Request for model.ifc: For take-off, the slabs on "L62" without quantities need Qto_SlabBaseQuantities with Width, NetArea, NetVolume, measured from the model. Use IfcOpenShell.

First a look at what the model holds.

```python
import ifcopenshell
import ifcopenshell.util.element
import ifcopenshell.util.unit

model = ifcopenshell.open("model.ifc")
print(model.schema)
for unit_type in ("LENGTHUNIT", "AREAUNIT", "VOLUMEUNIT"):
    print(unit_type, ifcopenshell.util.unit.calculate_unit_scale(model, unit_type))
storey = next(s for s in model.by_type("IfcBuildingStorey") if s.Name == "L62")
slabs = [e for e in ifcopenshell.util.element.get_decomposition(storey) if e.is_a("IfcSlab")]
for e in sorted(slabs, key=lambda e: e.id()):
    print(e.id(), e.is_a(), e.Name, list(ifcopenshell.util.element.get_psets(e, qtos_only=True)), sep=" | ")
```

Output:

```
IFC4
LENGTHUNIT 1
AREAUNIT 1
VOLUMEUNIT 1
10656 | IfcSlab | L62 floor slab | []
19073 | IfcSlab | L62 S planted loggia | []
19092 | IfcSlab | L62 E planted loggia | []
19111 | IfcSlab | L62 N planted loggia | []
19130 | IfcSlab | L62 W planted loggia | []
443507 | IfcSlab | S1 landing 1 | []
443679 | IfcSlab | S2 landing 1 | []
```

```python
import ifcopenshell
import ifcopenshell.api.pset
import ifcopenshell.geom
import ifcopenshell.util.element
import ifcopenshell.util.shape
import ifcopenshell.util.unit

model = ifcopenshell.open("model.ifc")
unit_scale = ifcopenshell.util.unit.calculate_unit_scale(model)
area_scale = ifcopenshell.util.unit.calculate_unit_scale(model, "AREAUNIT")
volume_scale = ifcopenshell.util.unit.calculate_unit_scale(model, "VOLUMEUNIT")
settings = ifcopenshell.geom.settings()

storey = next(s for s in model.by_type("IfcBuildingStorey") if s.Name == "L62")
slabs = [e for e in ifcopenshell.util.element.get_decomposition(storey) if e.is_a("IfcSlab")]

for e in sorted(slabs, key=lambda e: e.id()):
    if ifcopenshell.util.element.get_psets(e, qtos_only=True, should_inherit=False):
        continue
    # Geometry comes back in metres, in the element's own axes.
    shape = ifcopenshell.geom.create_shape(settings, e)
    values = {
        "Width": ifcopenshell.util.shape.get_z(shape.geometry) / unit_scale,
        "NetArea": ifcopenshell.util.shape.get_footprint_area(shape.geometry) / area_scale,
        "NetVolume": ifcopenshell.util.shape.get_volume(shape.geometry) / volume_scale,
    }
    qto = ifcopenshell.api.pset.add_qto(model, product=e, name="Qto_SlabBaseQuantities")
    ifcopenshell.api.pset.edit_qto(model, qto=qto, properties=values)
    print(e.id(), {k: round(v, 3) for k, v in values.items()})

model.write("model_updated.ifc")
```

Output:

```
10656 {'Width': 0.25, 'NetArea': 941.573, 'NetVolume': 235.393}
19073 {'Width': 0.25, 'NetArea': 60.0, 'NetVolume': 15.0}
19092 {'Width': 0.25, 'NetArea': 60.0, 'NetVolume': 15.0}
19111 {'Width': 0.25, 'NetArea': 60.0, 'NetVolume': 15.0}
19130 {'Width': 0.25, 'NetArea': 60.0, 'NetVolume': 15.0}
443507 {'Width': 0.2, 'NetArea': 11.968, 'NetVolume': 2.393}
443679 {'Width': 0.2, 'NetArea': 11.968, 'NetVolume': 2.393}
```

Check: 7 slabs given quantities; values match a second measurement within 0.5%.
